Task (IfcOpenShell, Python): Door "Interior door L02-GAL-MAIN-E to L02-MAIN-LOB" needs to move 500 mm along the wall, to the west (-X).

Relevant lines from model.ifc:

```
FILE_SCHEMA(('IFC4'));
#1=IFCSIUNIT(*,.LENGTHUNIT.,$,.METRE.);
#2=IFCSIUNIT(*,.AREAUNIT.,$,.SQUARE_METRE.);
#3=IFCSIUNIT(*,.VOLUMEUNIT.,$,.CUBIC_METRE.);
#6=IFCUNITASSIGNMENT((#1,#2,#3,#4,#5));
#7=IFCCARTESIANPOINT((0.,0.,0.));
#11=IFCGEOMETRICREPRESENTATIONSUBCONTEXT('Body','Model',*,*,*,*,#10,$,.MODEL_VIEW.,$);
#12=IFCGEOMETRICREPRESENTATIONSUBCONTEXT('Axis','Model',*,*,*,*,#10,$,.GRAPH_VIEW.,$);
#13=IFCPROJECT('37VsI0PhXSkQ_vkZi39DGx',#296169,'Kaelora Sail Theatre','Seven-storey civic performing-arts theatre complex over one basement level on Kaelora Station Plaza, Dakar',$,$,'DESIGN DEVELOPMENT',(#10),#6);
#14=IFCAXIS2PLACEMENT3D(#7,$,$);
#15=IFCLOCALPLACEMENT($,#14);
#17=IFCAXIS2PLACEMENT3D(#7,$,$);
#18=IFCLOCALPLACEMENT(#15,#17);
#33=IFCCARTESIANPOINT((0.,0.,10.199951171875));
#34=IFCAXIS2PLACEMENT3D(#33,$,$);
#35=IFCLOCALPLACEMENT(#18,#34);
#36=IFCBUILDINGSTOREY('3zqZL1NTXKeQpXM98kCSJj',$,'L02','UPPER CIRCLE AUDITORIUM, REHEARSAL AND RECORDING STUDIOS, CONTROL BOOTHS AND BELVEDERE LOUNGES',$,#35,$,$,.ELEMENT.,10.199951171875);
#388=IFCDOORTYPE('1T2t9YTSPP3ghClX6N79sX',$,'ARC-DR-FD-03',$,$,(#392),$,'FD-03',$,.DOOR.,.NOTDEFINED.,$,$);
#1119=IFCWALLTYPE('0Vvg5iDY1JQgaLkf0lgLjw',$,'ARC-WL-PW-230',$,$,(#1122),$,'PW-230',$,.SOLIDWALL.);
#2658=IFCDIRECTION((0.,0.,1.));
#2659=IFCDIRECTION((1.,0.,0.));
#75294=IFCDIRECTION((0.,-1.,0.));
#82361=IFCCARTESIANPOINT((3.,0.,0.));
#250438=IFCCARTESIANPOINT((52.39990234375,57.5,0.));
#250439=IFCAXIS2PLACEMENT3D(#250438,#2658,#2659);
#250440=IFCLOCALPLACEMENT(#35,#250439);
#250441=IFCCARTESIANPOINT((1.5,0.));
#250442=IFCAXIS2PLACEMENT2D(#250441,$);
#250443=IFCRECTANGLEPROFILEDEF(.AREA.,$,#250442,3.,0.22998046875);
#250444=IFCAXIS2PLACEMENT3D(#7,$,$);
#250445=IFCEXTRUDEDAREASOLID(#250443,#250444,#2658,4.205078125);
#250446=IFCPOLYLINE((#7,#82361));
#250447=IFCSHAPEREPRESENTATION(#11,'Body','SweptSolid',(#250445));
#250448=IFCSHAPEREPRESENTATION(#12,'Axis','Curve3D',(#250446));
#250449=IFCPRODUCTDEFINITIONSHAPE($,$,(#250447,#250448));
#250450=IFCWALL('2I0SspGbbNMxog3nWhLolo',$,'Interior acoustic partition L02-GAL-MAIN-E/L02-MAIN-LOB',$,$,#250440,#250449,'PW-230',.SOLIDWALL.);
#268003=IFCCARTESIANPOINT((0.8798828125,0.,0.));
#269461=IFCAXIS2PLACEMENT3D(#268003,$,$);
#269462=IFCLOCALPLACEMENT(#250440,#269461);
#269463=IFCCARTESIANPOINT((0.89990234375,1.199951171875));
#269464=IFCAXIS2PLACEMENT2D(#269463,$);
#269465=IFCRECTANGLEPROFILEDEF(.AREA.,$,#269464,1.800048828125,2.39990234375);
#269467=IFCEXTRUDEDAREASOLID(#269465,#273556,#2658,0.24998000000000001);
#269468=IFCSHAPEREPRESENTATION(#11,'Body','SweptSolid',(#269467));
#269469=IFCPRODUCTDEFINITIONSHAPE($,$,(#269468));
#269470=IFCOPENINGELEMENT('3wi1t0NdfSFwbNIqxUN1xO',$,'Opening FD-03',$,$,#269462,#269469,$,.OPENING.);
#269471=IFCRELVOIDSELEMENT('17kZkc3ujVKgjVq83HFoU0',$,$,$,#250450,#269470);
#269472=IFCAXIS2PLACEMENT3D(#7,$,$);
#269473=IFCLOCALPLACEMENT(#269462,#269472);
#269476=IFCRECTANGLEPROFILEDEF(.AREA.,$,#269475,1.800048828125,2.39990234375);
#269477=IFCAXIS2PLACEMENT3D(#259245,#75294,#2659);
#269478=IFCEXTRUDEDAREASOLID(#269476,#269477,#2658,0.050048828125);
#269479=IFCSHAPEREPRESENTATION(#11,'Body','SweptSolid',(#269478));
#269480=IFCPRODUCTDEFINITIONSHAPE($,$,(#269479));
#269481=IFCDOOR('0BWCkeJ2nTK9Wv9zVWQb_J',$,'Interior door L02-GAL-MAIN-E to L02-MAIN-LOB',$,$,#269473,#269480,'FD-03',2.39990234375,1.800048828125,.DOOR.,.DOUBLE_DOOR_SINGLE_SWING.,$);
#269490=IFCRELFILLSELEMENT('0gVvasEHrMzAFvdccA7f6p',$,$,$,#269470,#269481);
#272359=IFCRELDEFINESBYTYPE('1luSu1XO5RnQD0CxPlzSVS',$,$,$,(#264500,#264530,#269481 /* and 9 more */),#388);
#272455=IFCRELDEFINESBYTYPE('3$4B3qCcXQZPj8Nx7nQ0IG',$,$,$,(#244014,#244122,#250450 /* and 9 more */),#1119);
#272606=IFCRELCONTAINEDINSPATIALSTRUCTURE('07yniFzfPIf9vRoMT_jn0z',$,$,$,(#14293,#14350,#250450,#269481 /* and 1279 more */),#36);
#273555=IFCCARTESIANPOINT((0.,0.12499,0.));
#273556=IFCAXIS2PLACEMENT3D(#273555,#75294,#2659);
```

```python
import ifcopenshell
import ifcopenshell.api.geometry
import ifcopenshell.util.placement
import ifcopenshell.util.unit

model = ifcopenshell.open("model.ifc")
unit_scale = ifcopenshell.util.unit.calculate_unit_scale(model)

door = model.by_id(269481)
opening = door.FillsVoids[0].RelatingOpeningElement
wall = opening.VoidsElements[0].RelatingBuildingElement

wall_matrix = ifcopenshell.util.placement.get_local_placement(wall.ObjectPlacement)
shift = wall_matrix[:3, 0] * -0.5 / unit_scale
before = ifcopenshell.util.placement.get_local_placement(door.ObjectPlacement)[:3, 3].copy()

# The door is placed relative to its opening, so it follows when the opening moves.
matrix = ifcopenshell.util.placement.get_local_placement(opening.ObjectPlacement)
matrix[:3, 3] += shift
ifcopenshell.api.geometry.edit_object_placement(
    model, product=opening, matrix=matrix, is_si=False, should_transform_children=True
)

after = ifcopenshell.util.placement.get_local_placement(door.ObjectPlacement)[:3, 3]
print("door moved by", (after - before).round(3) + 0.0)

model.write("model_v2.ifc")
```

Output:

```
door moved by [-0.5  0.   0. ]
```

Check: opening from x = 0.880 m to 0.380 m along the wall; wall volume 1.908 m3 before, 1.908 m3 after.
